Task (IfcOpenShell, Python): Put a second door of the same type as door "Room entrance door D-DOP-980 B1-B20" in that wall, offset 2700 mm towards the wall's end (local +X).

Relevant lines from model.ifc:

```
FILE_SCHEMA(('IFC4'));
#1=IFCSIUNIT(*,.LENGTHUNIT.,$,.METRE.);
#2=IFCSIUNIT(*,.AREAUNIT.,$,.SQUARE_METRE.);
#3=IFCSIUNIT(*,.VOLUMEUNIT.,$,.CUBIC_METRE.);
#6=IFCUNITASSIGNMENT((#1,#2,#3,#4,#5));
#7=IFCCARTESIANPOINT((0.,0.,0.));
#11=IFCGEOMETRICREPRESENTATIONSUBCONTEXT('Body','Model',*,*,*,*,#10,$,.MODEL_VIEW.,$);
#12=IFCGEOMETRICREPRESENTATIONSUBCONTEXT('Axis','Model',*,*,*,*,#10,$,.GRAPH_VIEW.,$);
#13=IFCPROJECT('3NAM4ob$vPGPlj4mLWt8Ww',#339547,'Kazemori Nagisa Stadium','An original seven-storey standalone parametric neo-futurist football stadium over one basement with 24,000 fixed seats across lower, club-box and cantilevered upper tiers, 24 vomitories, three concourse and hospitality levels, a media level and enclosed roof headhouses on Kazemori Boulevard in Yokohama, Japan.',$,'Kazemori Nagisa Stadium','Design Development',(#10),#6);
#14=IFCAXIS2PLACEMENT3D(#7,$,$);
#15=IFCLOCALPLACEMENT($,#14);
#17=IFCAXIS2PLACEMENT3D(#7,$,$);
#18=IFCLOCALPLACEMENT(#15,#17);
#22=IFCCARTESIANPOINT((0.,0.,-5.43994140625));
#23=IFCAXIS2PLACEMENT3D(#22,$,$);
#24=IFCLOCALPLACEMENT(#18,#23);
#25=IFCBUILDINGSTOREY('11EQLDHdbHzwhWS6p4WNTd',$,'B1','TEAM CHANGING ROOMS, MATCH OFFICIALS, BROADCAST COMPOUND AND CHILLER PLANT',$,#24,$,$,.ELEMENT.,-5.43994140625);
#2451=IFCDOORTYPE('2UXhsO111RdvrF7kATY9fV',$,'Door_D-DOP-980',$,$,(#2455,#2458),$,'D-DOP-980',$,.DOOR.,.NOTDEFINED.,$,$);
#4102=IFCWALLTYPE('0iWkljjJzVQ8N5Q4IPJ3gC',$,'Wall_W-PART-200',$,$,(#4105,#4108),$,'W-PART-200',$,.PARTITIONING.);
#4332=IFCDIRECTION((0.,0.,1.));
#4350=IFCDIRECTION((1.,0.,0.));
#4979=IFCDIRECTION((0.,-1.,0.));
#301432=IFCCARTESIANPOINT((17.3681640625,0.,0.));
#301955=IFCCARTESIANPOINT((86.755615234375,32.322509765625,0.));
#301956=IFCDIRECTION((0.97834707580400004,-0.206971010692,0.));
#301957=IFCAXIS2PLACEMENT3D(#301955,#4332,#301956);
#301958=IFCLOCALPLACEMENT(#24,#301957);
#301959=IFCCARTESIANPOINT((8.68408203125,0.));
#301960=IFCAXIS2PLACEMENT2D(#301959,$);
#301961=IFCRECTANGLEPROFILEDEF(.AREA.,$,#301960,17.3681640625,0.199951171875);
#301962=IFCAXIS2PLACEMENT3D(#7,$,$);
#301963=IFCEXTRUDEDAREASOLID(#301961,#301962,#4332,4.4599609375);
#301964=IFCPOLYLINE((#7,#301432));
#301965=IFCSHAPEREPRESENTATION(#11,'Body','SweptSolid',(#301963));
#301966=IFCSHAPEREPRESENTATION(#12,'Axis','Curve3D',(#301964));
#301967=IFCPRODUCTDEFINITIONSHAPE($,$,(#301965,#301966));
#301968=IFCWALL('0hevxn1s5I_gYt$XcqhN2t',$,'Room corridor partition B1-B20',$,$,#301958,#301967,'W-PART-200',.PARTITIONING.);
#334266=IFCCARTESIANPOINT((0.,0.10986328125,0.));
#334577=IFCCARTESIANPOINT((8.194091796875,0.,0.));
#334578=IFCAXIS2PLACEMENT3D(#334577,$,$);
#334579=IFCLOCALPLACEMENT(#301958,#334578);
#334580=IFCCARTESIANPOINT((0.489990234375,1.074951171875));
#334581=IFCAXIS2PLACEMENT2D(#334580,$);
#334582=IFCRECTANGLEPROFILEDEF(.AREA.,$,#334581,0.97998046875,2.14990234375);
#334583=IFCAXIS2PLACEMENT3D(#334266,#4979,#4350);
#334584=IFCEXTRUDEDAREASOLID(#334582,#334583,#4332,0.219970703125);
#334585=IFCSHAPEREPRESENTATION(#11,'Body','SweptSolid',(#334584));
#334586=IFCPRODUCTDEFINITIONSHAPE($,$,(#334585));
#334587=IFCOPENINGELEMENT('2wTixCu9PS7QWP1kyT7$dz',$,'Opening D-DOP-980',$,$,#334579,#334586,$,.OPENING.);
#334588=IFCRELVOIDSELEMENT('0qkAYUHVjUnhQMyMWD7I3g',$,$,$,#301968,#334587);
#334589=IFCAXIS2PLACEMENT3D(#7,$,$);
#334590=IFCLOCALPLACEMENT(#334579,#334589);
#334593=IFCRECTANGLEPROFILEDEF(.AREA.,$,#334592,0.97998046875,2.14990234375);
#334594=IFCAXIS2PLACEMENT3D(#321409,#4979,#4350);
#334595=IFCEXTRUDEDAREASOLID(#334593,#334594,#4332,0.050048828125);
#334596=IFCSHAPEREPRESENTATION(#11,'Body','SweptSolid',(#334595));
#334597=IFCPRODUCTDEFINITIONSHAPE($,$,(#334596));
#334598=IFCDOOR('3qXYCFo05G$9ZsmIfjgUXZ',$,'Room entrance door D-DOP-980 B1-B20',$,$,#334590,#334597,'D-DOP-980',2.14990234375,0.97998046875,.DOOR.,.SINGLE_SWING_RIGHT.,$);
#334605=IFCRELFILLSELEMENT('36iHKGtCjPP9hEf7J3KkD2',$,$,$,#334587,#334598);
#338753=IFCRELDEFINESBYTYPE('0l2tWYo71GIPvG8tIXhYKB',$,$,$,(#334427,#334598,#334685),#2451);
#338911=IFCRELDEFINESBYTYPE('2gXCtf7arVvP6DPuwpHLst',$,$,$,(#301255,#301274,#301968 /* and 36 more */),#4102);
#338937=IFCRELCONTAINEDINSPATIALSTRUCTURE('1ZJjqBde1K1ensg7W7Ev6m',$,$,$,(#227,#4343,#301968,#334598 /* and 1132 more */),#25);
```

```python
import ifcopenshell
import ifcopenshell.api.feature
import ifcopenshell.api.geometry
import ifcopenshell.api.root
import ifcopenshell.geom
import ifcopenshell.util.element
import ifcopenshell.util.placement
import ifcopenshell.util.shape
import ifcopenshell.util.unit

model = ifcopenshell.open("model.ifc")
unit_scale = ifcopenshell.util.unit.calculate_unit_scale(model)
settings = ifcopenshell.geom.settings()


def volume(element):
    """Net volume in cubic metres, openings subtracted."""
    shape = ifcopenshell.geom.create_shape(settings, element)
    return ifcopenshell.util.shape.get_volume(shape.geometry)


door = model.by_guid("3qXYCFo05G$9ZsmIfjgUXZ")
opening = door.FillsVoids[0].RelatingOpeningElement
wall = opening.VoidsElements[0].RelatingBuildingElement
before = volume(wall)
shift = ifcopenshell.util.placement.get_local_placement(wall.ObjectPlacement)[:3, 0] * 2.7 / unit_scale

# copy_class copies the void relationship, type, container and properties, but no geometry.
new_opening = ifcopenshell.api.root.copy_class(model, product=opening)
new_opening.Representation = ifcopenshell.util.element.copy_deep(
    model, opening.Representation, exclude=["IfcGeometricRepresentationContext", "IfcRepresentationMap"]
)
new_door = ifcopenshell.api.root.copy_class(model, product=door)
new_door.Representation = ifcopenshell.util.element.copy_deep(
    model, door.Representation, exclude=["IfcGeometricRepresentationContext", "IfcRepresentationMap"]
)
new_door.Tag = None
ifcopenshell.api.feature.add_filling(model, opening=new_opening, element=new_door)

for old, new in ((opening, new_opening), (door, new_door)):
    matrix = ifcopenshell.util.placement.get_local_placement(old.ObjectPlacement)
    matrix[:3, 3] += shift
    ifcopenshell.api.geometry.edit_object_placement(model, product=new, matrix=matrix, is_si=False)

after = volume(wall)

print(f"wall volume {before:.3f} -> {after:.3f} m3")

model.write("model_edited.ifc")
```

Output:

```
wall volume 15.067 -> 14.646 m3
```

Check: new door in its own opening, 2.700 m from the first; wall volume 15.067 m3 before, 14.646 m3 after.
